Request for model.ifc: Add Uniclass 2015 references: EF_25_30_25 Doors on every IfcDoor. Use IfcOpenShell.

First a look at what the model holds.

```python
import ifcopenshell

model = ifcopenshell.open("model.ifc")
print(model.schema)
print("classifications:", [c.Name for c in model.by_type("IfcClassification")])
for ifc_class in ("IfcDoor", "IfcRoof", "IfcStair", "IfcWall", "IfcWindow"):
    print(ifc_class, len(model.by_type(ifc_class)))
```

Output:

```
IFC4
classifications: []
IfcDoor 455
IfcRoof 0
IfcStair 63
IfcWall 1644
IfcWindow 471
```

```python
import ifcopenshell
import ifcopenshell.api.classification

model = ifcopenshell.open("model.ifc")

system = ifcopenshell.api.classification.add_classification(model, classification="Uniclass 2015")

codes = {
    "IfcDoor": ("EF_25_30_25", "Doors"),
}
for ifc_class, (code, name) in codes.items():
    products = model.by_type(ifc_class)
    ifcopenshell.api.classification.add_reference(
        model, products=products, classification=system, identification=code, name=name
    )
    print(code, len(products))

model.write("model_updated.ifc")
```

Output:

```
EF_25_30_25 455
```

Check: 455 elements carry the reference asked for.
